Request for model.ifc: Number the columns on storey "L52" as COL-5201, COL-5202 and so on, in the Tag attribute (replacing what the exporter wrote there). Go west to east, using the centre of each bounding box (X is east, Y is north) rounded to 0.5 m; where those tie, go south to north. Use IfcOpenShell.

First a look at what the model holds.

```python
import ifcopenshell
import ifcopenshell.util.element
import ifcopenshell.util.placement

model = ifcopenshell.open("model.ifc")
print(model.schema)
storey = next(s for s in model.by_type("IfcBuildingStorey") if s.Name == "L52")
columns = [e for e in ifcopenshell.util.element.get_decomposition(storey) if e.is_a("IfcColumn")]
for e in sorted(columns, key=lambda e: e.id()):
    origin = ifcopenshell.util.placement.get_local_placement(e.ObjectPlacement)[:3, 3]
    print(e.id(), e.Tag, e.Name, origin.round(2) + 0.0, sep=" | ")
```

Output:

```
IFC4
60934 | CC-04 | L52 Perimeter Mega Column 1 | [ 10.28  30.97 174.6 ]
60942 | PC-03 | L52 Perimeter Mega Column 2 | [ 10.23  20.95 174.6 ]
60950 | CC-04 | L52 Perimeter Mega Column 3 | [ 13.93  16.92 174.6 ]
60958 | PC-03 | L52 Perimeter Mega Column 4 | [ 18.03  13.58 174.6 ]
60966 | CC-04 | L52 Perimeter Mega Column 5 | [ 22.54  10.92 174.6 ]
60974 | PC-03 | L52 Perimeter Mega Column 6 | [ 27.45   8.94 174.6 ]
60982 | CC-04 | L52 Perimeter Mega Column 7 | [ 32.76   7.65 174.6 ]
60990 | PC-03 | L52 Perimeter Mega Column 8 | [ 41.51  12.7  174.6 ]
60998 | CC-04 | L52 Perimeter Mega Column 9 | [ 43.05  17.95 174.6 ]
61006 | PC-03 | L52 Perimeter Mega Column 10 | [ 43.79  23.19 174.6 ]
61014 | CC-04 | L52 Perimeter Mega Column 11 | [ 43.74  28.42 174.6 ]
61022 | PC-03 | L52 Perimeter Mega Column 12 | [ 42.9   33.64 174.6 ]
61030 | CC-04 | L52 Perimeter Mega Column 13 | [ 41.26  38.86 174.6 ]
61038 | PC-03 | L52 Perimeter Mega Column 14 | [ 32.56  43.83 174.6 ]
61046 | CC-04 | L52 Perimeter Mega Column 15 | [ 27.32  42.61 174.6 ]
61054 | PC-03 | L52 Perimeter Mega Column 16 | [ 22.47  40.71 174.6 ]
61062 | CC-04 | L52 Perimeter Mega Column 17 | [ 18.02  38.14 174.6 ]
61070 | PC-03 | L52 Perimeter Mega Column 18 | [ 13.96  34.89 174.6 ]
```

```python
import ifcopenshell
import ifcopenshell.geom
import ifcopenshell.util.element
import ifcopenshell.util.shape

model = ifcopenshell.open("model.ifc")
settings = ifcopenshell.geom.settings()
settings.set("use-world-coords", True)


def centre(element):
    shape = ifcopenshell.geom.create_shape(settings, element)
    return ifcopenshell.util.shape.get_bbox_centroid(shape.geometry)


storey = next(s for s in model.by_type("IfcBuildingStorey") if s.Name == "L52")
columns = [e for e in ifcopenshell.util.element.get_decomposition(storey) if e.is_a("IfcColumn")]

# Insertion points can sit at a corner or the storey origin, so sort by the geometry (in metres).
centres = {e: centre(e) for e in columns}
columns.sort(key=lambda e: (round(centres[e][0] / 0.5), centres[e][1]))

for i, e in enumerate(columns, start=1):
    number = f"COL-52{i:02d}"
    e.Tag = number
    print(e.id(), number)

model.write("model_rev.ifc")
```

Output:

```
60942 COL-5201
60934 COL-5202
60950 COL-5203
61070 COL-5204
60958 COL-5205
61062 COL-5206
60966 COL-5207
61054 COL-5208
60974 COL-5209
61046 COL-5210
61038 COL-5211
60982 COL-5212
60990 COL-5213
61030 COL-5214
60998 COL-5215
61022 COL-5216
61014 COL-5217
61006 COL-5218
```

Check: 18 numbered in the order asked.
